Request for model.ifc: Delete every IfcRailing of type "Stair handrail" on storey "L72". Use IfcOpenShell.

First a look at what the model holds.

```python
import ifcopenshell
import ifcopenshell.util.element

model = ifcopenshell.open("model.ifc")
print(model.schema)
storey = next(s for s in model.by_type("IfcBuildingStorey") if s.Name == "L72")
railings = [e for e in ifcopenshell.util.element.get_decomposition(storey) if e.is_a("IfcRailing")]
seen = {}
for e in railings:
    element_type = ifcopenshell.util.element.get_type(e)
    name = element_type.Name if element_type not in (None, e) else None
    seen[name] = seen.get(name, 0) + 1
for name, count in sorted(seen.items(), key=str):
    print(count, "x", name)
```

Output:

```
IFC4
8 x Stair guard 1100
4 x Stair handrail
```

```python
import ifcopenshell
import ifcopenshell.api.root
import ifcopenshell.util.element

model = ifcopenshell.open("model.ifc")

storey = next(s for s in model.by_type("IfcBuildingStorey") if s.Name == "L72")
railings = [e for e in ifcopenshell.util.element.get_decomposition(storey) if e.is_a("IfcRailing")]
targets = [e for e in railings if (t := ifcopenshell.util.element.get_type(e)) not in (None, e) and t.Name == "Stair handrail"]

for e in targets:
    ifcopenshell.api.root.remove_product(model, product=e)
print(len(targets), "removed")

model.write("model_v2.ifc")
```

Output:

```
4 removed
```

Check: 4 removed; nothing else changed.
